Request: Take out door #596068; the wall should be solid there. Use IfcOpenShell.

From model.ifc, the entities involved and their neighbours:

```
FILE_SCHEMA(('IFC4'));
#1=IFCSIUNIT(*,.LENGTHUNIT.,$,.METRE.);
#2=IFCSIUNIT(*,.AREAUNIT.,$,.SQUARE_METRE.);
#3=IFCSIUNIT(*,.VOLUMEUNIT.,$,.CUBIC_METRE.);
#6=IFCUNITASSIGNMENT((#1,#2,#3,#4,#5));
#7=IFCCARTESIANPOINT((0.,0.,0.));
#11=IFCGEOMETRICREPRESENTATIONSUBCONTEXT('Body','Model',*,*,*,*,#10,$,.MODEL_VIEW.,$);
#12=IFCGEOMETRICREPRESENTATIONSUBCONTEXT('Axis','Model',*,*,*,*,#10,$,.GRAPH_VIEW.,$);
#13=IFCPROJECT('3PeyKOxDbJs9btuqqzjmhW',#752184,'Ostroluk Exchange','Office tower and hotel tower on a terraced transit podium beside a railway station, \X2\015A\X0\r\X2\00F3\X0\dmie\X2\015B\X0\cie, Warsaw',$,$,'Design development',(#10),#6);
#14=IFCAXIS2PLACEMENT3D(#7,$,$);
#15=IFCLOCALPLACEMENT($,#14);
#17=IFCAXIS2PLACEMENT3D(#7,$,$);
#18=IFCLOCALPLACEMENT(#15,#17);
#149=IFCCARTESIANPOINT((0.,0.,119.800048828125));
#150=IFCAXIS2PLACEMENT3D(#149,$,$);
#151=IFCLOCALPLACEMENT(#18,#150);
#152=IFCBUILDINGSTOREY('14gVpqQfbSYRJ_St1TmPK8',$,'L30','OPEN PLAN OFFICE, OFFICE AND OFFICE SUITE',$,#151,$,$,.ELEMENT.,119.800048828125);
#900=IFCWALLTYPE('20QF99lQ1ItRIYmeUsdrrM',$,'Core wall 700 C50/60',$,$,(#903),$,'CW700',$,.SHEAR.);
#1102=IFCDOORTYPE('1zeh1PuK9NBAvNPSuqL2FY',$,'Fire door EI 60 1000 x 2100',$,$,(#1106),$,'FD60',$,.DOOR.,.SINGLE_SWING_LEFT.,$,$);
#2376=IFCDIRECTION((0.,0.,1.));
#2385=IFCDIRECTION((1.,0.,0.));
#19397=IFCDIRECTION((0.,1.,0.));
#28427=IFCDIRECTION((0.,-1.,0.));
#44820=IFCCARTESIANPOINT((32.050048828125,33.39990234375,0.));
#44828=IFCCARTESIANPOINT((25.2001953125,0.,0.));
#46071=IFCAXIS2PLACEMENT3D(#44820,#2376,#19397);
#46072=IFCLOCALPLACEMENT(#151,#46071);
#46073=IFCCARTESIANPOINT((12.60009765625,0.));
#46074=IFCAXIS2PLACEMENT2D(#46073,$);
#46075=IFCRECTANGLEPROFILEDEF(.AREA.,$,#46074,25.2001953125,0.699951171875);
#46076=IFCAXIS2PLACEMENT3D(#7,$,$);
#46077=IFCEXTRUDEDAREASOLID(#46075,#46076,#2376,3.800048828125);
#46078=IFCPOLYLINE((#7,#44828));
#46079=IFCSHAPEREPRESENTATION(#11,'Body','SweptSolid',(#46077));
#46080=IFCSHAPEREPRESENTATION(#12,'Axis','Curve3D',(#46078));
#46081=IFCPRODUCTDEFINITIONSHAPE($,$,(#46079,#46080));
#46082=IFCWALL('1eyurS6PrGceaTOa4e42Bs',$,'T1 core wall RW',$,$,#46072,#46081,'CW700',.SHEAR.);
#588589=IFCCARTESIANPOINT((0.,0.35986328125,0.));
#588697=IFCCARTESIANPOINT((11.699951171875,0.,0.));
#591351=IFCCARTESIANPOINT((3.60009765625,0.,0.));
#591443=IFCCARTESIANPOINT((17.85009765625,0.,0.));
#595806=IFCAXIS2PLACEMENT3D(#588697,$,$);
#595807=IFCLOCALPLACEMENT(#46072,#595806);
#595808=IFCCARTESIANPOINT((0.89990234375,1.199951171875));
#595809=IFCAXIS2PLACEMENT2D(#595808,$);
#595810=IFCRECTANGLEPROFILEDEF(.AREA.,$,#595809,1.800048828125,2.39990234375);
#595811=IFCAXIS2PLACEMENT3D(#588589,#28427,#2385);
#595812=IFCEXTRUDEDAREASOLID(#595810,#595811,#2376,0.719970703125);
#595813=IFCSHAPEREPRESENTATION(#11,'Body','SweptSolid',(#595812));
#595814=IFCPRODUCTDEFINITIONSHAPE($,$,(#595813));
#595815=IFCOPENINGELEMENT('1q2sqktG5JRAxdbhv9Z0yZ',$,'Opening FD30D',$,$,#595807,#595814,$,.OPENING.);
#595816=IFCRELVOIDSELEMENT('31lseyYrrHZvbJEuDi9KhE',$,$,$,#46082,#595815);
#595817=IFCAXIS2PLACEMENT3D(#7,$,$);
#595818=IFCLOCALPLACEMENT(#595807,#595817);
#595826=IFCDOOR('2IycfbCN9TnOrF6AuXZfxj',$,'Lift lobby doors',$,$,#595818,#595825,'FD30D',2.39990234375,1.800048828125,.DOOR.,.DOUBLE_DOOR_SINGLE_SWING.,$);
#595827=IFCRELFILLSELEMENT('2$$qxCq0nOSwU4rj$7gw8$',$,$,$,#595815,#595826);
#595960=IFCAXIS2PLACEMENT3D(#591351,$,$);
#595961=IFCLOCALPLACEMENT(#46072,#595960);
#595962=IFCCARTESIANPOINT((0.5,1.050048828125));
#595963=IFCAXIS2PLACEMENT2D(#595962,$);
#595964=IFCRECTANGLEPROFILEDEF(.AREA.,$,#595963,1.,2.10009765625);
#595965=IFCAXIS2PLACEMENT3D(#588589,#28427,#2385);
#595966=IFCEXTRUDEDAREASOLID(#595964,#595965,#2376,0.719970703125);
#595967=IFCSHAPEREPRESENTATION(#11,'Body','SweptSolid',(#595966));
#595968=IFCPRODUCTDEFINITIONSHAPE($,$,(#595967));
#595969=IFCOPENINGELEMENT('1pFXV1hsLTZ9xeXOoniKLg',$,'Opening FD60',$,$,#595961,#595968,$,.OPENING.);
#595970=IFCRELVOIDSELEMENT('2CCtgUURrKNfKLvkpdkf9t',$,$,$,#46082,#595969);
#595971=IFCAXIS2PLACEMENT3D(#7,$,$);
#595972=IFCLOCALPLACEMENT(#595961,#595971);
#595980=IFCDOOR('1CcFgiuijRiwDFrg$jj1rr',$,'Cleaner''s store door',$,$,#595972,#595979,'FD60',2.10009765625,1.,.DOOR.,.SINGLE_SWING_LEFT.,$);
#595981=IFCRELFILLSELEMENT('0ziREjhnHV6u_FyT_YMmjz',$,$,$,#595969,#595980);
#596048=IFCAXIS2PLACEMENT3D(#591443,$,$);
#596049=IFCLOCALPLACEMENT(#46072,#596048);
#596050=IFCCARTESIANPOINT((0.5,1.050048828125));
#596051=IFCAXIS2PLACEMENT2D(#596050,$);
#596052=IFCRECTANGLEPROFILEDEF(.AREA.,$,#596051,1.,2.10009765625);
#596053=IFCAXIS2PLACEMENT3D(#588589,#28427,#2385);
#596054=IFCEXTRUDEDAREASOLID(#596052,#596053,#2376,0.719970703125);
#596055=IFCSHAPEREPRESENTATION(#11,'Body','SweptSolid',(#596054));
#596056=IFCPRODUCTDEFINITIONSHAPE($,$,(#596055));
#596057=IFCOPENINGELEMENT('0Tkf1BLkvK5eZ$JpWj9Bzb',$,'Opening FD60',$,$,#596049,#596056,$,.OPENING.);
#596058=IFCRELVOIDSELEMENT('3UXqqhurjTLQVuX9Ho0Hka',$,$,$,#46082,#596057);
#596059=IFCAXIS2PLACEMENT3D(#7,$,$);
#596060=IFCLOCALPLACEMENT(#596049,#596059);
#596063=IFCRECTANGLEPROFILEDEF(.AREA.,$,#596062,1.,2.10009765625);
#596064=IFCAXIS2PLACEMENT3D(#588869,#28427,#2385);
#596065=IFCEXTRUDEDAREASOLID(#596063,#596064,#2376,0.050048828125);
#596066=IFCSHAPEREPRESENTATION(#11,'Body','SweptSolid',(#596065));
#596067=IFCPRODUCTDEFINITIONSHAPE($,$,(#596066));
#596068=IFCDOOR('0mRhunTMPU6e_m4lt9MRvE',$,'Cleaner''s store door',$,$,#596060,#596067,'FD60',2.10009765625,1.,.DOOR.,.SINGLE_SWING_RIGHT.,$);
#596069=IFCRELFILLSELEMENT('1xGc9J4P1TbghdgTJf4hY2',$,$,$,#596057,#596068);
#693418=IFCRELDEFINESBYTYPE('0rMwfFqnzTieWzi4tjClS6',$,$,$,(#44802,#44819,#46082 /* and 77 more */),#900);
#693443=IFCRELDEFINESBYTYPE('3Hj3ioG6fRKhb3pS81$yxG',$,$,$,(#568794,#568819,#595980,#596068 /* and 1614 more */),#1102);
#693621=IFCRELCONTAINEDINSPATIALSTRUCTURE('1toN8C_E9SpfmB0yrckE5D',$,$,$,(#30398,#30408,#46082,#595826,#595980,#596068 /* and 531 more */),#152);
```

```python
import ifcopenshell
import ifcopenshell.api.feature
import ifcopenshell.api.root
import ifcopenshell.geom
import ifcopenshell.util.shape

model = ifcopenshell.open("model.ifc")
settings = ifcopenshell.geom.settings()


def volume(element):
    """Net volume in cubic metres, openings subtracted."""
    shape = ifcopenshell.geom.create_shape(settings, element)
    return ifcopenshell.util.shape.get_volume(shape.geometry)


door = model.by_guid("0mRhunTMPU6e_m4lt9MRvE")
opening = door.FillsVoids[0].RelatingOpeningElement
wall = opening.VoidsElements[0].RelatingBuildingElement
before = volume(wall)

ifcopenshell.api.root.remove_product(model, product=door)
ifcopenshell.api.feature.remove_feature(model, feature=opening)

after = volume(wall)

print(f"wall volume {before:.3f} -> {after:.3f} m3")

model.write("model_v2.ifc")
```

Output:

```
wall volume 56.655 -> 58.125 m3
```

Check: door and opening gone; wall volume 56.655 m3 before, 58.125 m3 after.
